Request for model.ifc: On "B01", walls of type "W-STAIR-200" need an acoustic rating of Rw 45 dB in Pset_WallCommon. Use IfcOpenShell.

First a look at what the model holds.

```python
import ifcopenshell
import ifcopenshell.util.element

model = ifcopenshell.open("model.ifc")
print(model.schema)
storey = next(s for s in model.by_type("IfcBuildingStorey") if s.Name == "B01")
walls = [e for e in ifcopenshell.util.element.get_decomposition(storey) if e.is_a("IfcWall")]
seen = {}
for e in walls:
    element_type = ifcopenshell.util.element.get_type(e)
    key = (element_type.Name if element_type != e and element_type else None, ifcopenshell.util.element.get_pset(e, "Pset_WallCommon", "AcousticRating"))
    seen[key] = seen.get(key, 0) + 1
for (name, value), count in sorted(seen.items(), key=str):
    print(count, "x", name, "|", value)
```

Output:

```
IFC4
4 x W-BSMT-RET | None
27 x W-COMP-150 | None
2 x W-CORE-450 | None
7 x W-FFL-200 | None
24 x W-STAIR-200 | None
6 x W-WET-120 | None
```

```python
import ifcopenshell
import ifcopenshell.api.pset
import ifcopenshell.util.element

model = ifcopenshell.open("model.ifc")

storey = next(s for s in model.by_type("IfcBuildingStorey") if s.Name == "B01")
walls = [e for e in ifcopenshell.util.element.get_decomposition(storey) if e.is_a("IfcWall")]

count = 0
for e in walls:
    element_type = ifcopenshell.util.element.get_type(e)
    if element_type in (None, e) or element_type.Name != "W-STAIR-200":
        continue
    found = ifcopenshell.util.element.get_pset(e, "Pset_WallCommon", should_inherit=False)
    if found:
        pset = model.by_id(found["id"])
        if len(ifcopenshell.util.element.get_elements_by_pset(pset)) > 1:
            pset = ifcopenshell.api.pset.unshare_pset(model, products=[e], pset=pset)[0]
    else:
        pset = ifcopenshell.api.pset.add_pset(model, product=e, name="Pset_WallCommon")
    ifcopenshell.api.pset.edit_pset(model, pset=pset, properties={"AcousticRating": "Rw 45 dB"})
    count += 1

print(count, "walls updated")

model.write("model_v2.ifc")
```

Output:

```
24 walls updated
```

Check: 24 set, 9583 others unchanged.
